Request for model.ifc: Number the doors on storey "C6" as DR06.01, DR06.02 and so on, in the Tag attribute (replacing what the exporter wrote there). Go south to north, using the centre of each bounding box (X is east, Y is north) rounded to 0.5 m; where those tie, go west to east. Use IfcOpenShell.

First a look at what the model holds.

```python
import ifcopenshell
import ifcopenshell.util.element
import ifcopenshell.util.placement

model = ifcopenshell.open("model.ifc")
print(model.schema)
storey = next(s for s in model.by_type("IfcBuildingStorey") if s.Name == "C6")
doors = [e for e in ifcopenshell.util.element.get_decomposition(storey) if e.is_a("IfcDoor")]
for e in sorted(doors, key=lambda e: e.id()):
    origin = ifcopenshell.util.placement.get_local_placement(e.ObjectPlacement)[:3, 3]
    print(e.id(), e.Tag, e.Name, origin.round(2) + 0.0, sep=" | ")
```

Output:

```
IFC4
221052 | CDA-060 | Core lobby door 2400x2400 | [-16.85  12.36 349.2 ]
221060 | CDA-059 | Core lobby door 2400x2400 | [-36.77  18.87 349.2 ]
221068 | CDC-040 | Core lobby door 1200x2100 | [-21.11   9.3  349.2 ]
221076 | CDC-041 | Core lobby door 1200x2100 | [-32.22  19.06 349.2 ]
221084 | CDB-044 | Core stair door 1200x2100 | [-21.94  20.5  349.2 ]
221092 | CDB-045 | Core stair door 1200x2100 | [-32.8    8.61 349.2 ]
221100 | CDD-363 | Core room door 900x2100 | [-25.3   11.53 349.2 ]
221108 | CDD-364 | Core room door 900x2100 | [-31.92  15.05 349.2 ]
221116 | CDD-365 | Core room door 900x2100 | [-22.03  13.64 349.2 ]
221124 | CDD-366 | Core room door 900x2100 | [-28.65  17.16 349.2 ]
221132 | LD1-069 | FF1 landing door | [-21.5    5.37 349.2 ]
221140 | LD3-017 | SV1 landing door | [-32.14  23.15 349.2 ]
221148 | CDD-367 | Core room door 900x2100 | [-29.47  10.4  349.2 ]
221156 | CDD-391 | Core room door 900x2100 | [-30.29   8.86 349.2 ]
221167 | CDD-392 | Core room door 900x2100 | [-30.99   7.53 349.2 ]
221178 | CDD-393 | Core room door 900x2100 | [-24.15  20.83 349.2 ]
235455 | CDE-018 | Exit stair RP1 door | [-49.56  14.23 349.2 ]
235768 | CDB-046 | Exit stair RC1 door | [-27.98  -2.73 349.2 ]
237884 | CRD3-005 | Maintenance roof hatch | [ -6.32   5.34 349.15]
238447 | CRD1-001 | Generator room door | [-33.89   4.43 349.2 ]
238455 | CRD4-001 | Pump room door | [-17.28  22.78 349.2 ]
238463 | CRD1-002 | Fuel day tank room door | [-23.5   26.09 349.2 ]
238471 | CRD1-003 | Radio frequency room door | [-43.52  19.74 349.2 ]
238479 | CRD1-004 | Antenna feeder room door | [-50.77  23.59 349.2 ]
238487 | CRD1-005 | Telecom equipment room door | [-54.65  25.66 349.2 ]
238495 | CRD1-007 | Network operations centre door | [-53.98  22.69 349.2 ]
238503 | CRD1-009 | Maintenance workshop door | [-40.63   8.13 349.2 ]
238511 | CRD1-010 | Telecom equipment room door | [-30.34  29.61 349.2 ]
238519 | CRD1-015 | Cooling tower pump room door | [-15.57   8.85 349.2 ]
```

```python
import ifcopenshell
import ifcopenshell.geom
import ifcopenshell.util.element
import ifcopenshell.util.shape

model = ifcopenshell.open("model.ifc")
settings = ifcopenshell.geom.settings()
settings.set("use-world-coords", True)


def centre(element):
    shape = ifcopenshell.geom.create_shape(settings, element)
    return ifcopenshell.util.shape.get_bbox_centroid(shape.geometry)


storey = next(s for s in model.by_type("IfcBuildingStorey") if s.Name == "C6")
doors = [e for e in ifcopenshell.util.element.get_decomposition(storey) if e.is_a("IfcDoor")]

# Insertion points can sit at a corner or the storey origin, so sort by the geometry (in metres).
centres = {e: centre(e) for e in doors}
doors.sort(key=lambda e: (round(centres[e][1] / 0.5), centres[e][0]))

for i, e in enumerate(doors, start=1):
    number = f"DR06.{i:02d}"
    e.Tag = number
    print(e.id(), number)

model.write("model-out.ifc")
```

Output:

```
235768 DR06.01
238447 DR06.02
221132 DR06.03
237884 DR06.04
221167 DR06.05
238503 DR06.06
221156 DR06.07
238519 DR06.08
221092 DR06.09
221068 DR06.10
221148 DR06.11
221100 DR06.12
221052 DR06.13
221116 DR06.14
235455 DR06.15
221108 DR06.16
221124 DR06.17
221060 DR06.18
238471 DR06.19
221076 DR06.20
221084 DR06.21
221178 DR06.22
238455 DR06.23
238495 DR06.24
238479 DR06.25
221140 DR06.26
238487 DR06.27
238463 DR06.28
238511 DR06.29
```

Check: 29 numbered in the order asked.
